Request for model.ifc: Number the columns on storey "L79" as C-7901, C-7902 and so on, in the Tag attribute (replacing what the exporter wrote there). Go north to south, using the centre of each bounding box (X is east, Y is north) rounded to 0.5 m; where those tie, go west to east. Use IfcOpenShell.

First a look at what the model holds.

```python
import ifcopenshell
import ifcopenshell.util.element
import ifcopenshell.util.placement

model = ifcopenshell.open("model.ifc")
print(model.schema)
storey = next(s for s in model.by_type("IfcBuildingStorey") if s.Name == "L79")
columns = [e for e in ifcopenshell.util.element.get_decomposition(storey) if e.is_a("IfcColumn")]
for e in sorted(columns, key=lambda e: e.id()):
    origin = ifcopenshell.util.placement.get_local_placement(e.ObjectPlacement)[:3, 3]
    print(e.id(), e.Tag, e.Name, origin.round(2) + 0.0, sep=" | ")
```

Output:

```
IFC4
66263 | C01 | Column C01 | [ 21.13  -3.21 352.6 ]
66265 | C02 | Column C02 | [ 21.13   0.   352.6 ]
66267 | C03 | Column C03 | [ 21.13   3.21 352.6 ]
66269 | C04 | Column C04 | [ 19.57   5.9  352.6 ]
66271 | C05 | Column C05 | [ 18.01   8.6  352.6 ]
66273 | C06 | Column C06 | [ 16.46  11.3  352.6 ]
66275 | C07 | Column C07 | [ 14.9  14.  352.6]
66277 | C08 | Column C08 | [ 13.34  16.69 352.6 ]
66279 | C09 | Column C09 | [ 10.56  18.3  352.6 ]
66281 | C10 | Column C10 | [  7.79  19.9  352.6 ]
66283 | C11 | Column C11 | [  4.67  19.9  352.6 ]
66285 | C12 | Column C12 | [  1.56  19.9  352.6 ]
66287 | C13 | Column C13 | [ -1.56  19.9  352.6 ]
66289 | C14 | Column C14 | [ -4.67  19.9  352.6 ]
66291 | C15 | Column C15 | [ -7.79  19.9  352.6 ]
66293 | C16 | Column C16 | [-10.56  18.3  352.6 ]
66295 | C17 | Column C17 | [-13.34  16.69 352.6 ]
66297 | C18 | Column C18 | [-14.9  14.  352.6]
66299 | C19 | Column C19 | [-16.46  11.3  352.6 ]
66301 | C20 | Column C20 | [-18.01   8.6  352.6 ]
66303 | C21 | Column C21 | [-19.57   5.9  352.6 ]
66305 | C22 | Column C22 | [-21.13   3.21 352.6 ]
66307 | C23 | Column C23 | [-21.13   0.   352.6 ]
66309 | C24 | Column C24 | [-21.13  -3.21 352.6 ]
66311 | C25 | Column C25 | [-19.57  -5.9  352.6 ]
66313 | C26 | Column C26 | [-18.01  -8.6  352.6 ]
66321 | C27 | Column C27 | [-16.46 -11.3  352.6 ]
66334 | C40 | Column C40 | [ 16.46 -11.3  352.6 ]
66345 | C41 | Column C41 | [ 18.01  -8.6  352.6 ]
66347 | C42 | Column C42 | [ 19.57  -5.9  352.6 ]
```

```python
import ifcopenshell
import ifcopenshell.geom
import ifcopenshell.util.element
import ifcopenshell.util.shape

model = ifcopenshell.open("model.ifc")
settings = ifcopenshell.geom.settings()
settings.set("use-world-coords", True)


def centre(element):
    shape = ifcopenshell.geom.create_shape(settings, element)
    return ifcopenshell.util.shape.get_bbox_centroid(shape.geometry)


storey = next(s for s in model.by_type("IfcBuildingStorey") if s.Name == "L79")
columns = [e for e in ifcopenshell.util.element.get_decomposition(storey) if e.is_a("IfcColumn")]

# Insertion points can sit at a corner or the storey origin, so sort by the geometry (in metres).
centres = {e: centre(e) for e in columns}
columns.sort(key=lambda e: (-round(centres[e][1] / 0.5), centres[e][0]))

for i, e in enumerate(columns, start=1):
    number = f"C-79{i:02d}"
    e.Tag = number
    print(e.id(), number)

model.write("model_v2.ifc")
```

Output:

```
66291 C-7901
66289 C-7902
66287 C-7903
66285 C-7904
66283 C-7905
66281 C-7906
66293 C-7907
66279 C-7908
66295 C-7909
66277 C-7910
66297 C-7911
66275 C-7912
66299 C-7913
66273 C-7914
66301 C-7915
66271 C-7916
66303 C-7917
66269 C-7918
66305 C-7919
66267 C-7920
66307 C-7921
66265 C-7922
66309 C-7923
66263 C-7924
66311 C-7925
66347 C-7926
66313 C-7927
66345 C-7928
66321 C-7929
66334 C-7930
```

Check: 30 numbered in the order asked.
